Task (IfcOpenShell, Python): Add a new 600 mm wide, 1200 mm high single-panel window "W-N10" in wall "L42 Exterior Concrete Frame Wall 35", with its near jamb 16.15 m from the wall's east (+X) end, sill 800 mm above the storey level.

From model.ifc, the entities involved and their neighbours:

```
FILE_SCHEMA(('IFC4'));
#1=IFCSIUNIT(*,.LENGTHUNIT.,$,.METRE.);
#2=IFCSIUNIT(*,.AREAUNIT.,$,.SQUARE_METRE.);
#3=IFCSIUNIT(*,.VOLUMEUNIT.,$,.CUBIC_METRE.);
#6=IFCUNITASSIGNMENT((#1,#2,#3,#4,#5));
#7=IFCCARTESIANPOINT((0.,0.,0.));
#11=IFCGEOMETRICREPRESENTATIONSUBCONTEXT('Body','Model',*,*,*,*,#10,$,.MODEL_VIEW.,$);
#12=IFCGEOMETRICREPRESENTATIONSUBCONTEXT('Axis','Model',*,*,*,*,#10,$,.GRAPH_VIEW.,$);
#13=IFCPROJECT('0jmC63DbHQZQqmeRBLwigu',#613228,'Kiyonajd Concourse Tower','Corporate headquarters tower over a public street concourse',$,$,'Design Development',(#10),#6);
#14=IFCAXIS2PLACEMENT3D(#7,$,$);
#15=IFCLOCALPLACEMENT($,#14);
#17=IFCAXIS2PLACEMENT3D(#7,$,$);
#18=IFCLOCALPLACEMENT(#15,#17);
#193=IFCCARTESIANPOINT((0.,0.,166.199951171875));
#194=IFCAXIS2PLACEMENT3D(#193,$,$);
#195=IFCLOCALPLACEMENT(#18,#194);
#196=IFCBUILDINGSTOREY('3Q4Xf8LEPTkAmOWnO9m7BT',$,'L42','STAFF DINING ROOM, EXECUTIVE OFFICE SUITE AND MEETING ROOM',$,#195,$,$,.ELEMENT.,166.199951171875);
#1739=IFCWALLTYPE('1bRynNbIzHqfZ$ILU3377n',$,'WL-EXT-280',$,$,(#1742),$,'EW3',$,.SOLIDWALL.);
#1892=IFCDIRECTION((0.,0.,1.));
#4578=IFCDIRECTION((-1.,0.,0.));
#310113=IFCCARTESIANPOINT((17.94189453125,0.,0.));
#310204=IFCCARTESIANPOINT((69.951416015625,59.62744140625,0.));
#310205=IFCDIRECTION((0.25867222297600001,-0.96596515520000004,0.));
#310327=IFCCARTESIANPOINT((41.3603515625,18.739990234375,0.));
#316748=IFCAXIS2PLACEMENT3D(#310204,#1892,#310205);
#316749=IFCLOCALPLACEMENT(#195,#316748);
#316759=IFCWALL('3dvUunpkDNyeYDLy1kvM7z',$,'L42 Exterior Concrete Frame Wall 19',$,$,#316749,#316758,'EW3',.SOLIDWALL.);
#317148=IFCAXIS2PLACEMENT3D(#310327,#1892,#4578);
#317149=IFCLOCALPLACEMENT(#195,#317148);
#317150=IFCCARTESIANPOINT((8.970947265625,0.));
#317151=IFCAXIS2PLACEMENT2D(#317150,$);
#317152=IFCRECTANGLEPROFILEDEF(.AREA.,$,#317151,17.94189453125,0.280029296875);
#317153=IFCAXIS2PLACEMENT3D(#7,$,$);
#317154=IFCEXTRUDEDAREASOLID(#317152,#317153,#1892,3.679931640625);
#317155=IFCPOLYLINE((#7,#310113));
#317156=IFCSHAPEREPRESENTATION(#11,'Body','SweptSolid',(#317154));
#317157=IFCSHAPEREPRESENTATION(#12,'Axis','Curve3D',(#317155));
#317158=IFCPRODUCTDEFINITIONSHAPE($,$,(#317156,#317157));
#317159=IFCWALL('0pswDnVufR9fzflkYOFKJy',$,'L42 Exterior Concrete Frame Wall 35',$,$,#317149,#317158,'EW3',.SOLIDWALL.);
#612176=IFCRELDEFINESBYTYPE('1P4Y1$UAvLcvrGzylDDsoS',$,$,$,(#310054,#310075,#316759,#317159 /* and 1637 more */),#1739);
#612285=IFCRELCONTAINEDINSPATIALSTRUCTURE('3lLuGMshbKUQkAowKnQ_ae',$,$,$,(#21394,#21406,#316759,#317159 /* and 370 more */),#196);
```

```python
import numpy as np
import ifcopenshell
import ifcopenshell.api.feature
import ifcopenshell.api.geometry
import ifcopenshell.api.root
import ifcopenshell.api.spatial
import ifcopenshell.geom
import ifcopenshell.util.element
import ifcopenshell.util.placement
import ifcopenshell.util.representation
import ifcopenshell.util.shape
import ifcopenshell.util.unit

model = ifcopenshell.open("model.ifc")
unit_scale = ifcopenshell.util.unit.calculate_unit_scale(model)
settings = ifcopenshell.geom.settings()


def volume(element):
    """Net volume in cubic metres, openings subtracted."""
    shape = ifcopenshell.geom.create_shape(settings, element)
    return ifcopenshell.util.shape.get_volume(shape.geometry)


wall = model.by_guid("0pswDnVufR9fzflkYOFKJy")
storey = ifcopenshell.util.element.get_container(wall, ifc_class="IfcBuildingStorey")
context = ifcopenshell.util.representation.get_context(model, "Model", "Body", "MODEL_VIEW")
before = volume(wall)

width, height, from_end, sill = 0.6, 1.2, 16.15, 0.8  # metres

# The wall runs along its own X axis, and the end named is its -X end.
wall_shape = ifcopenshell.geom.create_shape(settings, wall)
x, y, z = ifcopenshell.util.shape.get_vertices(wall_shape.geometry).T
start = x.min() + from_end
face, thickness = float(y.min()), float(y.max() - y.min())
wall_matrix = ifcopenshell.util.placement.get_local_placement(wall.ObjectPlacement)
level = ifcopenshell.util.placement.get_local_placement(storey.ObjectPlacement)[2, 3]


def in_wall(x, y):
    """Placement at x, y metres in the wall's axes, at sill height."""
    matrix = wall_matrix.copy()
    matrix[:, 3] = wall_matrix @ np.array([x / unit_scale, y / unit_scale, 0.0, 1.0])
    matrix[2, 3] = level + sill / unit_scale
    return matrix


# Opening: a box that overshoots both wall faces by 50 mm.
opening = ifcopenshell.api.root.create_entity(model, ifc_class="IfcOpeningElement", predefined_type="OPENING")
box = ifcopenshell.api.geometry.add_wall_representation(
    model, context=context, length=width, height=height, thickness=thickness + 0.1
)
ifcopenshell.api.geometry.assign_representation(model, product=opening, representation=box)
ifcopenshell.api.geometry.edit_object_placement(model, product=opening, matrix=in_wall(start, face - 0.05), is_si=False)
ifcopenshell.api.feature.add_feature(model, feature=opening, element=wall)

window = ifcopenshell.api.root.create_entity(model, ifc_class="IfcWindow", name="W-N10", predefined_type="WINDOW")
window.OverallWidth, window.OverallHeight = width / unit_scale, height / unit_scale
window.PartitioningType = "SINGLE_PANEL"
body = ifcopenshell.api.geometry.add_window_representation(
    model,
    context=context,
    overall_width=window.OverallWidth,
    overall_height=window.OverallHeight,
    partition_type="SINGLE_PANEL",
)
ifcopenshell.api.geometry.assign_representation(model, product=window, representation=body)
ifcopenshell.api.spatial.assign_container(model, products=[window], relating_structure=storey)
ifcopenshell.api.feature.add_filling(model, opening=opening, element=window)

# Centre the window in the wall's thickness.
ifcopenshell.api.geometry.edit_object_placement(model, product=window, matrix=in_wall(start, face), is_si=False)
window_shape = ifcopenshell.geom.create_shape(settings, window)
depth = ifcopenshell.util.shape.get_vertices(window_shape.geometry)[:, 1]
offset = face + thickness / 2 - (depth.min() + depth.max()) / 2
ifcopenshell.api.geometry.edit_object_placement(model, product=window, matrix=in_wall(start, offset), is_si=False)

after = volume(wall)

print(f"wall volume {before:.3f} -> {after:.3f} m3")

model.write("model_edited.ifc")
```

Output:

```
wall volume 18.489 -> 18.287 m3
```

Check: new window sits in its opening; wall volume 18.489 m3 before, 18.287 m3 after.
